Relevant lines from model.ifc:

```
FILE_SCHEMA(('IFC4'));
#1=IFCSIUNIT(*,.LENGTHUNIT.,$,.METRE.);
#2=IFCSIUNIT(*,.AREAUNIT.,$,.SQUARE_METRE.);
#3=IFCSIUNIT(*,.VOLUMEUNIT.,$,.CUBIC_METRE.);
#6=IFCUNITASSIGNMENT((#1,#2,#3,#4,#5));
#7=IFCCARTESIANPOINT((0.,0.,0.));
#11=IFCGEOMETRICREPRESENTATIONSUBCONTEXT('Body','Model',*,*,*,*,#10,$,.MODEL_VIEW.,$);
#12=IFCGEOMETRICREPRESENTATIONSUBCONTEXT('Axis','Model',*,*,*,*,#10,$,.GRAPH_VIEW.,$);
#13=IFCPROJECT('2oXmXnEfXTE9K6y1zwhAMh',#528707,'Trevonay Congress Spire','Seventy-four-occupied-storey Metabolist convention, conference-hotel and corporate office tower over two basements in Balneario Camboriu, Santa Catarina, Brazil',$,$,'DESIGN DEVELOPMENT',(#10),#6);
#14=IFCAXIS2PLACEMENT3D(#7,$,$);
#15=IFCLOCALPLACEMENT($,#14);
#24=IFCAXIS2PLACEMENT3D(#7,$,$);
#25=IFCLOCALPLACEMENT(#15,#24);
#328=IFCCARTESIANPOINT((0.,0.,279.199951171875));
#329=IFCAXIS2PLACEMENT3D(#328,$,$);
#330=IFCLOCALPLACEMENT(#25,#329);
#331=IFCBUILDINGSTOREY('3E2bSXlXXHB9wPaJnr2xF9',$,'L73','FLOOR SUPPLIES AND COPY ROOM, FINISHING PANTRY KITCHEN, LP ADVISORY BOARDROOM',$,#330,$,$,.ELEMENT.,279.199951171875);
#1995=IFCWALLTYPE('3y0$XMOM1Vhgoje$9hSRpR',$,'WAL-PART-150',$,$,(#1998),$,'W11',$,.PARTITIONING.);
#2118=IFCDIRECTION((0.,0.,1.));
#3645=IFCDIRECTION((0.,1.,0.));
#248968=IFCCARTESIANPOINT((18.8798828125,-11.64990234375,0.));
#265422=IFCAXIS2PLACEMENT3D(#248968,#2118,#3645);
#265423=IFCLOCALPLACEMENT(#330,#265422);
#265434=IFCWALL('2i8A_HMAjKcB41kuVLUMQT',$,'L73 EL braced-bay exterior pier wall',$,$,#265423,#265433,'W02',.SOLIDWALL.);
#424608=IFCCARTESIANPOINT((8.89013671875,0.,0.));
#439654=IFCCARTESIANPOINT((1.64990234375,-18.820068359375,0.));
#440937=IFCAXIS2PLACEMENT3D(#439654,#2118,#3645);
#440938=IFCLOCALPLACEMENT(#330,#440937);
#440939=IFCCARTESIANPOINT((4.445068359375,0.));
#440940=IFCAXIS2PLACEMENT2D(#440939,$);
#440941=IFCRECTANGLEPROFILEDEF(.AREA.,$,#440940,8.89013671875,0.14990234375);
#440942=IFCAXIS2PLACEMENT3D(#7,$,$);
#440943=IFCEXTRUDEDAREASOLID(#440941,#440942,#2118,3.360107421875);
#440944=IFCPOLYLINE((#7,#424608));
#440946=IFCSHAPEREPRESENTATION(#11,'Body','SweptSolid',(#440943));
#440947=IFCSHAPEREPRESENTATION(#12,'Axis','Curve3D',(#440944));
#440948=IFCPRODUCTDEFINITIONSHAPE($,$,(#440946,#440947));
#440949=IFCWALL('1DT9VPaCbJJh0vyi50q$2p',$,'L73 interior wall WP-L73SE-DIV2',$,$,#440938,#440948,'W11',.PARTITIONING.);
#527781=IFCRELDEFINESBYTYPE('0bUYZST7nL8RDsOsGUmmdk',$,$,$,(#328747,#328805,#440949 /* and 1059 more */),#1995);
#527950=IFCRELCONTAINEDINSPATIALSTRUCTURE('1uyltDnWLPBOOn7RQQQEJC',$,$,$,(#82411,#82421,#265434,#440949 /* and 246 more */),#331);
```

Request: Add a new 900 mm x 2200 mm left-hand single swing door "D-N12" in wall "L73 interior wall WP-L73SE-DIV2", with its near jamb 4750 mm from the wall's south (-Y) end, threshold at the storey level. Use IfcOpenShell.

```python
import numpy as np
import ifcopenshell
import ifcopenshell.api.feature
import ifcopenshell.api.geometry
import ifcopenshell.api.root
import ifcopenshell.api.spatial
import ifcopenshell.geom
import ifcopenshell.util.element
import ifcopenshell.util.placement
import ifcopenshell.util.representation
import ifcopenshell.util.shape
import ifcopenshell.util.unit

model = ifcopenshell.open("model.ifc")
unit_scale = ifcopenshell.util.unit.calculate_unit_scale(model)
settings = ifcopenshell.geom.settings()


def volume(element):
    """Net volume in cubic metres, openings subtracted."""
    shape = ifcopenshell.geom.create_shape(settings, element)
    return ifcopenshell.util.shape.get_volume(shape.geometry)


wall = model.by_guid("1DT9VPaCbJJh0vyi50q$2p")
storey = ifcopenshell.util.element.get_container(wall, ifc_class="IfcBuildingStorey")
context = ifcopenshell.util.representation.get_context(model, "Model", "Body", "MODEL_VIEW")
before = volume(wall)

width, height, from_end, sill = 0.9, 2.2, 4.75, 0.0  # metres

# The wall runs along its own X axis, and the end named is its -X end.
wall_shape = ifcopenshell.geom.create_shape(settings, wall)
x, y, z = ifcopenshell.util.shape.get_vertices(wall_shape.geometry).T
start = x.min() + from_end
face, thickness = float(y.min()), float(y.max() - y.min())
wall_matrix = ifcopenshell.util.placement.get_local_placement(wall.ObjectPlacement)
level = ifcopenshell.util.placement.get_local_placement(storey.ObjectPlacement)[2, 3]


def in_wall(x, y):
    """Placement at x, y metres in the wall's axes, at sill height."""
    matrix = wall_matrix.copy()
    matrix[:, 3] = wall_matrix @ np.array([x / unit_scale, y / unit_scale, 0.0, 1.0])
    matrix[2, 3] = level + sill / unit_scale
    return matrix


# Opening: a box that overshoots both wall faces by 50 mm.
opening = ifcopenshell.api.root.create_entity(model, ifc_class="IfcOpeningElement", predefined_type="OPENING")
box = ifcopenshell.api.geometry.add_wall_representation(
    model, context=context, length=width, height=height, thickness=thickness + 0.1
)
ifcopenshell.api.geometry.assign_representation(model, product=opening, representation=box)
ifcopenshell.api.geometry.edit_object_placement(model, product=opening, matrix=in_wall(start, face - 0.05), is_si=False)
ifcopenshell.api.feature.add_feature(model, feature=opening, element=wall)

door = ifcopenshell.api.root.create_entity(model, ifc_class="IfcDoor", name="D-N12", predefined_type="DOOR")
door.OverallWidth, door.OverallHeight = width / unit_scale, height / unit_scale
door.OperationType = "SINGLE_SWING_LEFT"
body = ifcopenshell.api.geometry.add_door_representation(
    model,
    context=context,
    overall_width=door.OverallWidth,
    overall_height=door.OverallHeight,
    operation_type="SINGLE_SWING_LEFT",
    lining_properties={"LiningDepth": thickness / unit_scale, "ThresholdDepth": thickness / unit_scale},
)
ifcopenshell.api.geometry.assign_representation(model, product=door, representation=body)
ifcopenshell.api.spatial.assign_container(model, products=[door], relating_structure=storey)
ifcopenshell.api.feature.add_filling(model, opening=opening, element=door)

# The lining spans the wall, so the door starts at the wall face.
ifcopenshell.api.geometry.edit_object_placement(model, product=door, matrix=in_wall(start, face), is_si=False)

after = volume(wall)

print(f"wall volume {before:.3f} -> {after:.3f} m3")

model.write("model_updated.ifc")
```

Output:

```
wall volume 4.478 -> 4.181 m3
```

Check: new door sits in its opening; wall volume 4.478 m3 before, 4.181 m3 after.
